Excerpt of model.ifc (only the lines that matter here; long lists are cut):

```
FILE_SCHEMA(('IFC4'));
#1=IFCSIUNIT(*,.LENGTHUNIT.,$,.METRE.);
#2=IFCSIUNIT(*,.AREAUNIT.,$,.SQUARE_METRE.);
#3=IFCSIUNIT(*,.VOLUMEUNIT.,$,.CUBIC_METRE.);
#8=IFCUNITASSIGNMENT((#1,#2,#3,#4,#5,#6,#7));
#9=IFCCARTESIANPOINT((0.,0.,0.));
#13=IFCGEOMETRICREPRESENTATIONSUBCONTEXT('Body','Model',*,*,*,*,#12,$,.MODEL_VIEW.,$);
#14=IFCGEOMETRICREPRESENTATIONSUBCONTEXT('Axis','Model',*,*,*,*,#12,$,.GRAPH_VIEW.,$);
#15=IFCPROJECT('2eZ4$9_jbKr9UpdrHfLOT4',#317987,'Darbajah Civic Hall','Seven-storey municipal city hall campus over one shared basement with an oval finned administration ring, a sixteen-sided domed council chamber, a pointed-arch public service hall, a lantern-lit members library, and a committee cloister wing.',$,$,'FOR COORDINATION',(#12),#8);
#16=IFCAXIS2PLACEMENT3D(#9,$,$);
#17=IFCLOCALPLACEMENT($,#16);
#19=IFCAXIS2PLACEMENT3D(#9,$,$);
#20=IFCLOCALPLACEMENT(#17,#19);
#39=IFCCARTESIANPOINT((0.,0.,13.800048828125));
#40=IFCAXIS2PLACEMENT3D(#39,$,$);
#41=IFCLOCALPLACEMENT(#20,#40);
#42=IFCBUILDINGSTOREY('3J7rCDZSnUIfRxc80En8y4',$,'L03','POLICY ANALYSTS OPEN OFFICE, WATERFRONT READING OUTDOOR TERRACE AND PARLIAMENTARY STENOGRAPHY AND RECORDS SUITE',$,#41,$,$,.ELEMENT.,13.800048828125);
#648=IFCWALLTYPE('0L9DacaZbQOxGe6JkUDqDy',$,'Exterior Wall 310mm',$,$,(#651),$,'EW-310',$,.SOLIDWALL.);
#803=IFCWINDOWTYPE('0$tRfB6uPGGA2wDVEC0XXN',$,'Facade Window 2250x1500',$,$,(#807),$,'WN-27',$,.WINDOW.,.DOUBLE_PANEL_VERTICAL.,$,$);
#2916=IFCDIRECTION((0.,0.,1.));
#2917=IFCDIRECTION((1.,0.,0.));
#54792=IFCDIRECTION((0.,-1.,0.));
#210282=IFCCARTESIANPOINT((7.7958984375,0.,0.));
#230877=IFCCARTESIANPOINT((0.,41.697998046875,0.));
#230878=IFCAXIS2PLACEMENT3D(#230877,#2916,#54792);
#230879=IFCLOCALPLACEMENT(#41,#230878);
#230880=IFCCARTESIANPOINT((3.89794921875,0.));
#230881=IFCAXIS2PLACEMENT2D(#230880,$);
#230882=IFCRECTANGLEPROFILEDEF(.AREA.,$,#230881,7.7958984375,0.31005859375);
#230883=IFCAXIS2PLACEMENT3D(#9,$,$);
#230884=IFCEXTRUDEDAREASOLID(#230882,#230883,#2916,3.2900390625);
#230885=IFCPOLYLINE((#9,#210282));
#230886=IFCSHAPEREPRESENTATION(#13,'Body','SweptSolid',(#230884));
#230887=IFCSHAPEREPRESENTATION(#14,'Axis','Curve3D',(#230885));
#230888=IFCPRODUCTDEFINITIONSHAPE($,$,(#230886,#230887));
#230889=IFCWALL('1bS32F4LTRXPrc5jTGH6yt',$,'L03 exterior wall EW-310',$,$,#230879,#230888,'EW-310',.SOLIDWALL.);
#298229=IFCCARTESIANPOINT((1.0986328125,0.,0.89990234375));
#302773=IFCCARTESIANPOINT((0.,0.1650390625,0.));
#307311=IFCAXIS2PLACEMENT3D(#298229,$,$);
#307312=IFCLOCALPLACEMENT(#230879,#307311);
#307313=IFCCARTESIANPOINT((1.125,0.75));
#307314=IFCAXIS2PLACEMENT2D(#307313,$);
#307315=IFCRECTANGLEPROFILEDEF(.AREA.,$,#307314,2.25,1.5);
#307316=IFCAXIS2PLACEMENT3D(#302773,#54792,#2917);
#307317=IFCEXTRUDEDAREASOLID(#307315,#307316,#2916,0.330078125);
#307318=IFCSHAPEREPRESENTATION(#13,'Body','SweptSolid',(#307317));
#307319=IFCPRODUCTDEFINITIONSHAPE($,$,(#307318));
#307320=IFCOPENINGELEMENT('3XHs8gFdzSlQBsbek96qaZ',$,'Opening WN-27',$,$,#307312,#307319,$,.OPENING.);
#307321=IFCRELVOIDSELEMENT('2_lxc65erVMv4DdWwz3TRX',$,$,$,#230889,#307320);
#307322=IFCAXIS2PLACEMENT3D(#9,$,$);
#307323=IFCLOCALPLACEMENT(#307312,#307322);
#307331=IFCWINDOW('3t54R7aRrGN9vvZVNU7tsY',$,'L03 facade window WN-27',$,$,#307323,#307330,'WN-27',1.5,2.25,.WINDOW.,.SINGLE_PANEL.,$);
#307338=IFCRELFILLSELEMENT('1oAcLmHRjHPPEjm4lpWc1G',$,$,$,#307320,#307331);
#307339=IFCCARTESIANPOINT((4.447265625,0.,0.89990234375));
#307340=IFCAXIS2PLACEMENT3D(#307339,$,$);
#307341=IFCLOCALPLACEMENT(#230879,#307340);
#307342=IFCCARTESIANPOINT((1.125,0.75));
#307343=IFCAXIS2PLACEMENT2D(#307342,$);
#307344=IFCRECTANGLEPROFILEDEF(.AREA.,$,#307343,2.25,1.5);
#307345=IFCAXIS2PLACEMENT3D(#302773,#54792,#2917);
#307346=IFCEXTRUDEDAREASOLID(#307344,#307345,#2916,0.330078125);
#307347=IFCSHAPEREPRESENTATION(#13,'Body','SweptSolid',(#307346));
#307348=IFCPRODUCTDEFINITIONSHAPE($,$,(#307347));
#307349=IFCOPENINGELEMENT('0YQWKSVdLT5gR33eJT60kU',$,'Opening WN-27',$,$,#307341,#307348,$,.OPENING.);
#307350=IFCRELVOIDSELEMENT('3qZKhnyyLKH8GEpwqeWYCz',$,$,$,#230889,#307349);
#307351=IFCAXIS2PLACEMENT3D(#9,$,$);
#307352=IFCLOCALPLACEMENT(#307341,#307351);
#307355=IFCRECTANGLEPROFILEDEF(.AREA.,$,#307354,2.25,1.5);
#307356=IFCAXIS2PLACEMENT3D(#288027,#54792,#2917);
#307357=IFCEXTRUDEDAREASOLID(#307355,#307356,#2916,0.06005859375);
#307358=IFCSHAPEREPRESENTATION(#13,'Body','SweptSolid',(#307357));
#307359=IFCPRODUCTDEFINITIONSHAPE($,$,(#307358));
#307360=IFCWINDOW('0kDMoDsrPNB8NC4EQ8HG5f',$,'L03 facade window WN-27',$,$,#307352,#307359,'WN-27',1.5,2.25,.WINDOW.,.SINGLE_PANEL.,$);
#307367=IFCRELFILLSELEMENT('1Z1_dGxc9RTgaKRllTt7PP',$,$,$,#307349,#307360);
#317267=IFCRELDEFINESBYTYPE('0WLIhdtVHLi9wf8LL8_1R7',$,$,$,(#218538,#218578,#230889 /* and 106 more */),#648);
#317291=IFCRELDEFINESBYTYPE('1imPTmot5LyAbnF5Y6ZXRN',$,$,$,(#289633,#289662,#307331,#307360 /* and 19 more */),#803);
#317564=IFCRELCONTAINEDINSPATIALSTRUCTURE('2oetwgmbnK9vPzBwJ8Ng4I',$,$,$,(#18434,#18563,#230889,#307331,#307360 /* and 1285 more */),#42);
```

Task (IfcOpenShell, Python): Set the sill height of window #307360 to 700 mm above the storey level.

```python
import numpy as np
import ifcopenshell
import ifcopenshell.api.geometry
import ifcopenshell.geom
import ifcopenshell.util.element
import ifcopenshell.util.placement
import ifcopenshell.util.shape
import ifcopenshell.util.unit

model = ifcopenshell.open("model.ifc")
unit_scale = ifcopenshell.util.unit.calculate_unit_scale(model)

window = model.by_guid("0kDMoDsrPNB8NC4EQ8HG5f")
opening = window.FillsVoids[0].RelatingOpeningElement
storey = ifcopenshell.util.element.get_container(window, ifc_class="IfcBuildingStorey")
level = ifcopenshell.util.placement.get_local_placement(storey.ObjectPlacement)[2, 3]

# The opening's origin need not be at the sill, so measure its lowest point.
shape = ifcopenshell.geom.create_shape(ifcopenshell.geom.settings(), opening)
bottom = ifcopenshell.util.shape.get_shape_bottom_elevation(shape, shape.geometry) / unit_scale
dz = level + 0.7 / unit_scale - bottom

shift = np.array([0.0, 0.0, dz])
# The window is placed relative to its opening, so it follows when the opening moves.
matrix = ifcopenshell.util.placement.get_local_placement(opening.ObjectPlacement)
matrix[:3, 3] += shift
ifcopenshell.api.geometry.edit_object_placement(
    model, product=opening, matrix=matrix, is_si=False, should_transform_children=True
)

print(f"moved by {dz * unit_scale:+.3f} m")

model.write("model_rev.ifc")
```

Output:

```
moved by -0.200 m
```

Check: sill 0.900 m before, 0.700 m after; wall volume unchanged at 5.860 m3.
